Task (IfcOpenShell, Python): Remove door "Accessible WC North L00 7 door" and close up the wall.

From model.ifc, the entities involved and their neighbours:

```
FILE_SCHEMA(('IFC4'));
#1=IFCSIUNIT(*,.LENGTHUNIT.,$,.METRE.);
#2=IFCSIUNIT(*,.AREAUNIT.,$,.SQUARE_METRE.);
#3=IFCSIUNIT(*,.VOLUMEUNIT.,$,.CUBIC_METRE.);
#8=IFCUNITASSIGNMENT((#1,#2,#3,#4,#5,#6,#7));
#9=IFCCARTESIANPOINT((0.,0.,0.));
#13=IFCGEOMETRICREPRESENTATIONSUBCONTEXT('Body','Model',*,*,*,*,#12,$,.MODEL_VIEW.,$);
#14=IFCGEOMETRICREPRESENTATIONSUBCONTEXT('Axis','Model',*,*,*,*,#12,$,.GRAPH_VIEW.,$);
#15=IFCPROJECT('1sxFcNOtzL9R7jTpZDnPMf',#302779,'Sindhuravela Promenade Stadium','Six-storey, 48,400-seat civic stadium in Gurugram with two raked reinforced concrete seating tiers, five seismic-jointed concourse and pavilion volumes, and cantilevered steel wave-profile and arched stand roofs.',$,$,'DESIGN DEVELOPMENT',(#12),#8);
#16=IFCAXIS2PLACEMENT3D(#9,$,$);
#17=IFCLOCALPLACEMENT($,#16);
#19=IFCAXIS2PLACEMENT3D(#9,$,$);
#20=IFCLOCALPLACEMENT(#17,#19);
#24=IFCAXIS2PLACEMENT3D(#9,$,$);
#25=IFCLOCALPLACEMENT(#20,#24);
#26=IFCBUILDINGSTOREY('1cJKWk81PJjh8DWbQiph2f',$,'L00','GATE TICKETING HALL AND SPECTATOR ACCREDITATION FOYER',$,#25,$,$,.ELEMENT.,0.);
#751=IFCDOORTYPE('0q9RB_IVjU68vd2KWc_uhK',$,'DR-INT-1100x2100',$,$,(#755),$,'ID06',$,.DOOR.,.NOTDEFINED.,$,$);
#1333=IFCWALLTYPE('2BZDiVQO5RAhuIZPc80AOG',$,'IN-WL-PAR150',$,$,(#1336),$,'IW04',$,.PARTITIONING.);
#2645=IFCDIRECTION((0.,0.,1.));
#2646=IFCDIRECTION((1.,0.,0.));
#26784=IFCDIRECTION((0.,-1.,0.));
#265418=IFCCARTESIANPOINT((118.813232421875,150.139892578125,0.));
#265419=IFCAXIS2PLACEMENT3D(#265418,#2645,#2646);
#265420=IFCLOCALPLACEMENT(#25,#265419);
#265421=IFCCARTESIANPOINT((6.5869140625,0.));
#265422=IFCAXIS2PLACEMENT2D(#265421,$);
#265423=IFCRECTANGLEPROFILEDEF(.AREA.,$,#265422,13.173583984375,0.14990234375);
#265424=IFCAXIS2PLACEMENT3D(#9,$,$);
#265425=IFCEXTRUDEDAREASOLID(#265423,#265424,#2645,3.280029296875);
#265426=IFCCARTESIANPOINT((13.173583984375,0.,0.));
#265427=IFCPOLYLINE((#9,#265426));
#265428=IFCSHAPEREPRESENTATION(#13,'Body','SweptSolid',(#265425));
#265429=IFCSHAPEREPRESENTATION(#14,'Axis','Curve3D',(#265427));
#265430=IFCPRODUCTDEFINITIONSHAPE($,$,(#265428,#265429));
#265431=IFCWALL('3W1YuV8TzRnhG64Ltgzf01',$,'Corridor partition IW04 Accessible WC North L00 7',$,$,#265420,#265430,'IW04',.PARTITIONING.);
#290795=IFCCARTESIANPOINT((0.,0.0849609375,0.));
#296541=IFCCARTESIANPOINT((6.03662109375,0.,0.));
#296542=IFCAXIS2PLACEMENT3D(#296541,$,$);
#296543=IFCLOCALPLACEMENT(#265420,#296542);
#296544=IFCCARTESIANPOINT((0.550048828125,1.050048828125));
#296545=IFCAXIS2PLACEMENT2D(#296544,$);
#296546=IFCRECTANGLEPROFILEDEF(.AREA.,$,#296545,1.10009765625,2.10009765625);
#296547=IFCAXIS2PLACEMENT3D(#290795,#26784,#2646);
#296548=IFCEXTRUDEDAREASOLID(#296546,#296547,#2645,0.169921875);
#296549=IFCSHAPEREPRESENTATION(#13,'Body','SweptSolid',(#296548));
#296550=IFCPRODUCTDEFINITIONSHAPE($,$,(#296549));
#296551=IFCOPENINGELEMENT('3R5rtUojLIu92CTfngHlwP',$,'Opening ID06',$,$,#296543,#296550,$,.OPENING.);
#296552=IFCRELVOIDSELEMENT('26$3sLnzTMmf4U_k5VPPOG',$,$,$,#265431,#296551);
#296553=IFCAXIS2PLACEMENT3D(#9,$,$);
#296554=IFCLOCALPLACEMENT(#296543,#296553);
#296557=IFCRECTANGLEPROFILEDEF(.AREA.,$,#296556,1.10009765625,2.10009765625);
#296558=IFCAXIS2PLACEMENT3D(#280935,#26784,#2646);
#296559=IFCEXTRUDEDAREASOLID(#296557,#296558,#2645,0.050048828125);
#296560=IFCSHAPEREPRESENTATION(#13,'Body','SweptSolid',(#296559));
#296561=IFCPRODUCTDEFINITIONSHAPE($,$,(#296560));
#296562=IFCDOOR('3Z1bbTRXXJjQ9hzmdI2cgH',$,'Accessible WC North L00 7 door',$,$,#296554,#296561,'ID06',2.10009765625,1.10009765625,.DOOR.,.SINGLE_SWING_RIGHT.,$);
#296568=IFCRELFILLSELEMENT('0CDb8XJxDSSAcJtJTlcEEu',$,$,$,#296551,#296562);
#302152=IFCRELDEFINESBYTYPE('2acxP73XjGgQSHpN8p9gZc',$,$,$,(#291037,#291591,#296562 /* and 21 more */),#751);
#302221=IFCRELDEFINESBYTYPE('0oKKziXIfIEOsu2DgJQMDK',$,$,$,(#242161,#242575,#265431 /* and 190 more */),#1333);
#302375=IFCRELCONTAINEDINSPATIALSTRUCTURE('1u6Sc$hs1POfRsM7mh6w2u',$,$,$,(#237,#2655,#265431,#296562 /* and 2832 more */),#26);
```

```python
import ifcopenshell
import ifcopenshell.api.feature
import ifcopenshell.api.root
import ifcopenshell.geom
import ifcopenshell.util.shape

model = ifcopenshell.open("model.ifc")
settings = ifcopenshell.geom.settings()


def volume(element):
    """Net volume in cubic metres, openings subtracted."""
    shape = ifcopenshell.geom.create_shape(settings, element)
    return ifcopenshell.util.shape.get_volume(shape.geometry)


door = model.by_guid("3Z1bbTRXXJjQ9hzmdI2cgH")
opening = door.FillsVoids[0].RelatingOpeningElement
wall = opening.VoidsElements[0].RelatingBuildingElement
before = volume(wall)

ifcopenshell.api.root.remove_product(model, product=door)
ifcopenshell.api.feature.remove_feature(model, feature=opening)

after = volume(wall)

print(f"wall volume {before:.3f} -> {after:.3f} m3")

model.write("model_rev.ifc")
```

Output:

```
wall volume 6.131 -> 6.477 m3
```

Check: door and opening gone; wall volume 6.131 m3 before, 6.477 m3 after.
